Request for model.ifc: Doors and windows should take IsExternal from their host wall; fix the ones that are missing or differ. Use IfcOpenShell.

First a look at what the model holds.

```python
import ifcopenshell
import ifcopenshell.util.element

model = ifcopenshell.open("model.ifc")
print(model.schema)
seen = {}
for e in model.by_type("IfcDoor") + model.by_type("IfcWindow"):
    if not e.FillsVoids:
        continue
    host = e.FillsVoids[0].RelatingOpeningElement.VoidsElements[0].RelatingBuildingElement
    own = ifcopenshell.util.element.get_pset(e, f"Pset_{e.is_a()[3:].removesuffix('StandardCase')}Common", "IsExternal")
    wall = ifcopenshell.util.element.get_pset(host, "Pset_WallCommon", "IsExternal")
    seen[e.is_a(), own, wall] = seen.get((e.is_a(), own, wall), 0) + 1
for (cls, own, wall), count in sorted(seen.items(), key=str):
    print(count, cls, "IsExternal:", own, "| host wall:", wall)
```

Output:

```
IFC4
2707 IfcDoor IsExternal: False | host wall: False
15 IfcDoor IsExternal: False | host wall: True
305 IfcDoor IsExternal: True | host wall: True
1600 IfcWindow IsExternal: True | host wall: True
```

```python
import ifcopenshell
import ifcopenshell.api.pset
import ifcopenshell.util.element

model = ifcopenshell.open("model.ifc")

count = 0
for ifc_class, pset_name in (("IfcDoor", "Pset_DoorCommon"), ("IfcWindow", "Pset_WindowCommon")):
    for e in model.by_type(ifc_class):
        if not e.FillsVoids:
            continue
        host = e.FillsVoids[0].RelatingOpeningElement.VoidsElements[0].RelatingBuildingElement
        external = ifcopenshell.util.element.get_pset(host, "Pset_WallCommon", "IsExternal")
        if external is None or ifcopenshell.util.element.get_pset(e, pset_name, "IsExternal") == external:
            continue
        pset = ifcopenshell.api.pset.add_pset(model, product=e, name=pset_name)
        ifcopenshell.api.pset.edit_pset(model, pset=pset, properties={"IsExternal": external})
        count += 1

print(count, "updated")

model.write("model_edited.ifc")
```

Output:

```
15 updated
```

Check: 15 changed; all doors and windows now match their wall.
